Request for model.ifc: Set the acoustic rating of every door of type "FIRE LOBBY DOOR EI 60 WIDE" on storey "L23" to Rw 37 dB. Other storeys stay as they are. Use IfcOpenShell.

First a look at what the model holds.

```python
import ifcopenshell
import ifcopenshell.util.element

model = ifcopenshell.open("model.ifc")
print(model.schema)
storey = next(s for s in model.by_type("IfcBuildingStorey") if s.Name == "L23")
doors = [e for e in ifcopenshell.util.element.get_decomposition(storey) if e.is_a("IfcDoor")]
seen = {}
for e in doors:
    element_type = ifcopenshell.util.element.get_type(e)
    key = (element_type.Name if element_type != e and element_type else None, ifcopenshell.util.element.get_pset(e, "Pset_DoorCommon", "AcousticRating"))
    seen[key] = seen.get(key, 0) + 1
for (name, value), count in sorted(seen.items(), key=str):
    print(count, "x", name, "|", value)
```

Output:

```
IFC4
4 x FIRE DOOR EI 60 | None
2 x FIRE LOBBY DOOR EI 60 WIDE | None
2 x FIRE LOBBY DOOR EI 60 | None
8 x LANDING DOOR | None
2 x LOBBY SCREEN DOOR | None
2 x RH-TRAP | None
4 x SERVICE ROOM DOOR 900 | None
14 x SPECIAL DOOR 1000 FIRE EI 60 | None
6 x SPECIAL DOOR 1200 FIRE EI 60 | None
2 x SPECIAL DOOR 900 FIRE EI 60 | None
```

```python
import ifcopenshell
import ifcopenshell.api.pset
import ifcopenshell.util.element

model = ifcopenshell.open("model.ifc")

storey = next(s for s in model.by_type("IfcBuildingStorey") if s.Name == "L23")
doors = [e for e in ifcopenshell.util.element.get_decomposition(storey) if e.is_a("IfcDoor")]

count = 0
for e in doors:
    element_type = ifcopenshell.util.element.get_type(e)
    if element_type in (None, e) or element_type.Name != "FIRE LOBBY DOOR EI 60 WIDE":
        continue
    found = ifcopenshell.util.element.get_pset(e, "Pset_DoorCommon", should_inherit=False)
    if found:
        pset = model.by_id(found["id"])
        if len(ifcopenshell.util.element.get_elements_by_pset(pset)) > 1:
            pset = ifcopenshell.api.pset.unshare_pset(model, products=[e], pset=pset)[0]
    else:
        pset = ifcopenshell.api.pset.add_pset(model, product=e, name="Pset_DoorCommon")
    ifcopenshell.api.pset.edit_pset(model, pset=pset, properties={"AcousticRating": "Rw 37 dB"})
    count += 1

print(count, "doors updated")

model.write("model-out.ifc")
```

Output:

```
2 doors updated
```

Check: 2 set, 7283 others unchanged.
